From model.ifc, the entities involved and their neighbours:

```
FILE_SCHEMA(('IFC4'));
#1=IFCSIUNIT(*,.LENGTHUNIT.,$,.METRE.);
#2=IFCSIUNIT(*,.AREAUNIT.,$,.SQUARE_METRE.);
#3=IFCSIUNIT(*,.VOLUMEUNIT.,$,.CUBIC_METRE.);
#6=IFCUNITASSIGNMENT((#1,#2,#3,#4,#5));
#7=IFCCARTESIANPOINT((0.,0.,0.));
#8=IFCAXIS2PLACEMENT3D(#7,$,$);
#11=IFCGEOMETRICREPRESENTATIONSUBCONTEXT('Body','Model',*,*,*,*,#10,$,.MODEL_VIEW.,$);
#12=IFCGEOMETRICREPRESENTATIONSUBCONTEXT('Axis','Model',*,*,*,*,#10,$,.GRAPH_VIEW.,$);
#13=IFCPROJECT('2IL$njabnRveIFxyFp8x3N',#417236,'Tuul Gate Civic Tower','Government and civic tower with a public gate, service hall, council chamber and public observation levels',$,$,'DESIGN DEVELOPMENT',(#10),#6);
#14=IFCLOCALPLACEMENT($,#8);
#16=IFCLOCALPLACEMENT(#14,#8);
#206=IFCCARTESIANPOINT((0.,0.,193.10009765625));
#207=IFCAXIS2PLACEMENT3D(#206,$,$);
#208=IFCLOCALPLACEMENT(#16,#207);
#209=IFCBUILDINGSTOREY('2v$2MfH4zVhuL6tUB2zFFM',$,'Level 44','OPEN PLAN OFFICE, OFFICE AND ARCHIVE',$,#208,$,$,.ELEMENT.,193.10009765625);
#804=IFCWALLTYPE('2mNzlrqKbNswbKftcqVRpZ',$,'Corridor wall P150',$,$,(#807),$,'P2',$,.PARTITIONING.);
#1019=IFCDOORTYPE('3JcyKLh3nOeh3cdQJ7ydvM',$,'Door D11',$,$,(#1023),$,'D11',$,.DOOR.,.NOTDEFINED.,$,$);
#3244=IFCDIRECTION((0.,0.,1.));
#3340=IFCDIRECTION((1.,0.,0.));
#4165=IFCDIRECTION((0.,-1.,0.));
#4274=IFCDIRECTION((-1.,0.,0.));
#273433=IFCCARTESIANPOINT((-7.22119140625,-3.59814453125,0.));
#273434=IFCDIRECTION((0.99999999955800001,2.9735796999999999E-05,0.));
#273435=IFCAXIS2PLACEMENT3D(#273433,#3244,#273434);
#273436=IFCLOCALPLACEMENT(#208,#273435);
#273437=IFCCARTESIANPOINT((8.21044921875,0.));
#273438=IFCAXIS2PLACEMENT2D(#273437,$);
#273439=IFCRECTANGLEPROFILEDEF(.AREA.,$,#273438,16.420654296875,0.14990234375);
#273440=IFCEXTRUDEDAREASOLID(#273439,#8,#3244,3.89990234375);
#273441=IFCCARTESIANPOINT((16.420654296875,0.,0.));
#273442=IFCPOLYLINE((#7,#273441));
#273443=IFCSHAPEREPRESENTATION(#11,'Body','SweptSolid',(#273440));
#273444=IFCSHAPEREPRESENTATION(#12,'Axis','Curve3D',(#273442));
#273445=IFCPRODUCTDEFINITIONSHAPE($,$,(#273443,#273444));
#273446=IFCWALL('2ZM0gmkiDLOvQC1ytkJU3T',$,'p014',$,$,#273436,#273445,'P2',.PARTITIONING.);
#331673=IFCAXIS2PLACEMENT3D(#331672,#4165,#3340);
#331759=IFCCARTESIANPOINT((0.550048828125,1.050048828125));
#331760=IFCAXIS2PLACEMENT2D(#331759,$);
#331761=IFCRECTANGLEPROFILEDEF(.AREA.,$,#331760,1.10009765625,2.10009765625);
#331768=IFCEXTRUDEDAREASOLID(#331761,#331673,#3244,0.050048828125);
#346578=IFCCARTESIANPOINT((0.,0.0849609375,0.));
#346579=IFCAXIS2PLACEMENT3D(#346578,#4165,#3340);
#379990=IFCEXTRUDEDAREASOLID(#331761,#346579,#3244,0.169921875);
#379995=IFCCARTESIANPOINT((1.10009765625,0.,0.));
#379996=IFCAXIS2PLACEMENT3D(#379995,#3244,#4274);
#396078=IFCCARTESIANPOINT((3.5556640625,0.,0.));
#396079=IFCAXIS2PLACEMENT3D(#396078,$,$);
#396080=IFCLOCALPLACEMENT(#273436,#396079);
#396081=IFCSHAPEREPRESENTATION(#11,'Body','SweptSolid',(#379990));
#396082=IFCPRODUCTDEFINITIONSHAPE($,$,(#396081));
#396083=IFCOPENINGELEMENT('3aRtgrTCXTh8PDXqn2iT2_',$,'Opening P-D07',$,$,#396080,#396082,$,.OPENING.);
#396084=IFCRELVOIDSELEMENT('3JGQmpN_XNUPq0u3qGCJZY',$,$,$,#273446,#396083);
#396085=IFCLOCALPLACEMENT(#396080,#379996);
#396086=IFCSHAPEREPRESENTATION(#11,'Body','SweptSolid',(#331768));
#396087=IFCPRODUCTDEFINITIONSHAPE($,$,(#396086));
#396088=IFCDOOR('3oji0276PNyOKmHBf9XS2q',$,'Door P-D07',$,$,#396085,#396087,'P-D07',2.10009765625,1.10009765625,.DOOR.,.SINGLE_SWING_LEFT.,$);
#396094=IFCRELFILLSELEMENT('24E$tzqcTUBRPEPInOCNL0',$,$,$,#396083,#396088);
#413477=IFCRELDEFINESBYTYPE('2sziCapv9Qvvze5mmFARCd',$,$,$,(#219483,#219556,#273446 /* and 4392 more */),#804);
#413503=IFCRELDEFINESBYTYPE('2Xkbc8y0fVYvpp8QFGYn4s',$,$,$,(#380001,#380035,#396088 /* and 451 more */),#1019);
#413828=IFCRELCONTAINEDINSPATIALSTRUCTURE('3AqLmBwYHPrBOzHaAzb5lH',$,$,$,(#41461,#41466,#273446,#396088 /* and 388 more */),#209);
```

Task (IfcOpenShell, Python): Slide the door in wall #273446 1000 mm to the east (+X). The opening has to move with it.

```python
import ifcopenshell
import ifcopenshell.api.geometry
import ifcopenshell.util.placement

model = ifcopenshell.open("model.ifc")

door = model.by_guid("3oji0276PNyOKmHBf9XS2q")
opening = door.FillsVoids[0].RelatingOpeningElement
wall = opening.VoidsElements[0].RelatingBuildingElement

wall_matrix = ifcopenshell.util.placement.get_local_placement(wall.ObjectPlacement)
shift = wall_matrix[:3, 0] * 1.0
before = ifcopenshell.util.placement.get_local_placement(door.ObjectPlacement)[:3, 3].copy()

# The door is placed relative to its opening, so it follows when the opening moves.
matrix = ifcopenshell.util.placement.get_local_placement(opening.ObjectPlacement)
matrix[:3, 3] += shift
ifcopenshell.api.geometry.edit_object_placement(
    model, product=opening, matrix=matrix, is_si=False, should_transform_children=True
)

after = ifcopenshell.util.placement.get_local_placement(door.ObjectPlacement)[:3, 3]
print("door moved by", (after - before).round(3) + 0.0)

model.write("model_edited.ifc")
```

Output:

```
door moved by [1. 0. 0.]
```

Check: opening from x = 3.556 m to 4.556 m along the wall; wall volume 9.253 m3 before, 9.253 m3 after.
